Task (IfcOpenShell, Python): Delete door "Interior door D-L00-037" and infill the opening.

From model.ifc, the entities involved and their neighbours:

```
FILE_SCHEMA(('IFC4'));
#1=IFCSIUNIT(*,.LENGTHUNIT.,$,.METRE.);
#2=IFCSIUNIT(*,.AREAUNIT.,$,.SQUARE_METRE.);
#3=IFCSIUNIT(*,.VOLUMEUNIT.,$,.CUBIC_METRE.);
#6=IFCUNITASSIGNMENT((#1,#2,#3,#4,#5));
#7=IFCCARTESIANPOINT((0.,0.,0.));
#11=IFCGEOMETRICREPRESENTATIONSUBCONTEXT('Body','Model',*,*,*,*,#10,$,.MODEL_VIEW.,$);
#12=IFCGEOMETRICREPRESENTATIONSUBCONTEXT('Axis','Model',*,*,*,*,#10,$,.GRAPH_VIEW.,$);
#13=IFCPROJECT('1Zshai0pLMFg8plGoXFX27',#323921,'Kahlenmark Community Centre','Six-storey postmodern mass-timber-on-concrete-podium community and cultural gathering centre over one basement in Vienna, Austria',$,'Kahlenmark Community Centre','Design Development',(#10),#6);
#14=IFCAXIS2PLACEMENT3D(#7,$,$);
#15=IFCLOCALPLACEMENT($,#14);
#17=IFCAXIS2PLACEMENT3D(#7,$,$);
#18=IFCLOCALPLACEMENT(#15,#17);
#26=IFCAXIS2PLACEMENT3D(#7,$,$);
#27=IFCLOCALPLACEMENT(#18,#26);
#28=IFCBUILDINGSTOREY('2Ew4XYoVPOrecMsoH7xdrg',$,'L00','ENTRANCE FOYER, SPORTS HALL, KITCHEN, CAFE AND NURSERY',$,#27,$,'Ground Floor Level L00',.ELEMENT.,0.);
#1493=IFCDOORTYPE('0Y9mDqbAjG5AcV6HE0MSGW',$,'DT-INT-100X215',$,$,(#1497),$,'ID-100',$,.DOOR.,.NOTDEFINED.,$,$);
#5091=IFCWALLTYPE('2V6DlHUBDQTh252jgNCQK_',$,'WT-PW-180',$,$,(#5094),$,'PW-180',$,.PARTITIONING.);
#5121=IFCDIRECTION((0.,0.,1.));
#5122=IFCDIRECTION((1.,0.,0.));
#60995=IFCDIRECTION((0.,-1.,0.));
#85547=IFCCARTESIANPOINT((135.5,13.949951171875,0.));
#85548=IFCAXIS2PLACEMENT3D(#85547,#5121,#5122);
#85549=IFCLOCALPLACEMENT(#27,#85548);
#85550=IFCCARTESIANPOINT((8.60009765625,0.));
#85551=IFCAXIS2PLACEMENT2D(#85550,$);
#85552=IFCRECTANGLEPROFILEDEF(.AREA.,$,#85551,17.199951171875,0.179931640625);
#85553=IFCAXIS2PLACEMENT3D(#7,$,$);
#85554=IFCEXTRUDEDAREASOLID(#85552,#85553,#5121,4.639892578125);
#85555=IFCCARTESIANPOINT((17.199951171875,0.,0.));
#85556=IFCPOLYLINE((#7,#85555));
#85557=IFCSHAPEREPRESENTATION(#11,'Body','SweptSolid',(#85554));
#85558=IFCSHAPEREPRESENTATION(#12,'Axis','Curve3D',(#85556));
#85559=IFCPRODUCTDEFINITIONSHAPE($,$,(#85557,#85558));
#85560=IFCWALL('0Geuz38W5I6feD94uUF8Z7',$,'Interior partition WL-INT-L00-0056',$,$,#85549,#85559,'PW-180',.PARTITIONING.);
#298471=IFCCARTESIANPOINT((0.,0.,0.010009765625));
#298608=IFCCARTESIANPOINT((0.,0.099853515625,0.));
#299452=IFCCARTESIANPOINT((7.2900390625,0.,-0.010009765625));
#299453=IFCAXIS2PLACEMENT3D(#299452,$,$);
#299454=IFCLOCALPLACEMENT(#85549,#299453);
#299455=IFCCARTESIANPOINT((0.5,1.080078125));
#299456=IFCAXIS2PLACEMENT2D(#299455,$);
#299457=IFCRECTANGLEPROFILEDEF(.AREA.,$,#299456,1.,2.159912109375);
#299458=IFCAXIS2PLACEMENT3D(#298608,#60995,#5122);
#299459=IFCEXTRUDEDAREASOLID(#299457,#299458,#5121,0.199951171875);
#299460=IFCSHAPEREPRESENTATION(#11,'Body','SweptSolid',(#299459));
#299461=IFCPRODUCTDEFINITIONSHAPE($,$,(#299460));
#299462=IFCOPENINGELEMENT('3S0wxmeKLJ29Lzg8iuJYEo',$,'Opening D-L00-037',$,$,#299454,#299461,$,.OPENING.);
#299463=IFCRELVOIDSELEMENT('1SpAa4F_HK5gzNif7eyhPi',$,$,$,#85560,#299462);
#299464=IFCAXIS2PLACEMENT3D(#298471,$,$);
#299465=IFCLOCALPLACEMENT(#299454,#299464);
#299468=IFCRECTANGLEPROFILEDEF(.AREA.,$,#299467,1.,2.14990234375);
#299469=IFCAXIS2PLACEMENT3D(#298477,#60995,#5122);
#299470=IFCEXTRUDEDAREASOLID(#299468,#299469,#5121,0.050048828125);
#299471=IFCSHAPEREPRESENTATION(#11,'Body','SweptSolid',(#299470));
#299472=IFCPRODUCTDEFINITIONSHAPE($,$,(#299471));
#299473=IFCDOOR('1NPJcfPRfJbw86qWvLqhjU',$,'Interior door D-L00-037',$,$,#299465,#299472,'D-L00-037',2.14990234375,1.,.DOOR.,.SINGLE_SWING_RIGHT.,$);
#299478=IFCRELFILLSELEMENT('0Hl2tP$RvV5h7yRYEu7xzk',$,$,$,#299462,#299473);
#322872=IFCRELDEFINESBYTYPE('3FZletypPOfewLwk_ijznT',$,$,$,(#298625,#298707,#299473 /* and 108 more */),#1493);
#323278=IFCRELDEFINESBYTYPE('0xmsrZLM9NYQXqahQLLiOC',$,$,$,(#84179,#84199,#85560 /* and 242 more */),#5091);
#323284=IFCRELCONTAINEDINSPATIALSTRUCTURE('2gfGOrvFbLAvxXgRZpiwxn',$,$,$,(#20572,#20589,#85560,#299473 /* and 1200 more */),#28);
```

```python
import ifcopenshell
import ifcopenshell.api.feature
import ifcopenshell.api.root
import ifcopenshell.geom
import ifcopenshell.util.shape

model = ifcopenshell.open("model.ifc")
settings = ifcopenshell.geom.settings()


def volume(element):
    """Net volume in cubic metres, openings subtracted."""
    shape = ifcopenshell.geom.create_shape(settings, element)
    return ifcopenshell.util.shape.get_volume(shape.geometry)


door = model.by_id(299473)
opening = door.FillsVoids[0].RelatingOpeningElement
wall = opening.VoidsElements[0].RelatingBuildingElement
before = volume(wall)

ifcopenshell.api.root.remove_product(model, product=door)
ifcopenshell.api.feature.remove_feature(model, feature=opening)

after = volume(wall)

print(f"wall volume {before:.3f} -> {after:.3f} m3")

model.write("model_edited.ifc")
```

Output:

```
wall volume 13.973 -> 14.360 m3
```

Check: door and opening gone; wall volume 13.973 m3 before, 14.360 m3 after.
